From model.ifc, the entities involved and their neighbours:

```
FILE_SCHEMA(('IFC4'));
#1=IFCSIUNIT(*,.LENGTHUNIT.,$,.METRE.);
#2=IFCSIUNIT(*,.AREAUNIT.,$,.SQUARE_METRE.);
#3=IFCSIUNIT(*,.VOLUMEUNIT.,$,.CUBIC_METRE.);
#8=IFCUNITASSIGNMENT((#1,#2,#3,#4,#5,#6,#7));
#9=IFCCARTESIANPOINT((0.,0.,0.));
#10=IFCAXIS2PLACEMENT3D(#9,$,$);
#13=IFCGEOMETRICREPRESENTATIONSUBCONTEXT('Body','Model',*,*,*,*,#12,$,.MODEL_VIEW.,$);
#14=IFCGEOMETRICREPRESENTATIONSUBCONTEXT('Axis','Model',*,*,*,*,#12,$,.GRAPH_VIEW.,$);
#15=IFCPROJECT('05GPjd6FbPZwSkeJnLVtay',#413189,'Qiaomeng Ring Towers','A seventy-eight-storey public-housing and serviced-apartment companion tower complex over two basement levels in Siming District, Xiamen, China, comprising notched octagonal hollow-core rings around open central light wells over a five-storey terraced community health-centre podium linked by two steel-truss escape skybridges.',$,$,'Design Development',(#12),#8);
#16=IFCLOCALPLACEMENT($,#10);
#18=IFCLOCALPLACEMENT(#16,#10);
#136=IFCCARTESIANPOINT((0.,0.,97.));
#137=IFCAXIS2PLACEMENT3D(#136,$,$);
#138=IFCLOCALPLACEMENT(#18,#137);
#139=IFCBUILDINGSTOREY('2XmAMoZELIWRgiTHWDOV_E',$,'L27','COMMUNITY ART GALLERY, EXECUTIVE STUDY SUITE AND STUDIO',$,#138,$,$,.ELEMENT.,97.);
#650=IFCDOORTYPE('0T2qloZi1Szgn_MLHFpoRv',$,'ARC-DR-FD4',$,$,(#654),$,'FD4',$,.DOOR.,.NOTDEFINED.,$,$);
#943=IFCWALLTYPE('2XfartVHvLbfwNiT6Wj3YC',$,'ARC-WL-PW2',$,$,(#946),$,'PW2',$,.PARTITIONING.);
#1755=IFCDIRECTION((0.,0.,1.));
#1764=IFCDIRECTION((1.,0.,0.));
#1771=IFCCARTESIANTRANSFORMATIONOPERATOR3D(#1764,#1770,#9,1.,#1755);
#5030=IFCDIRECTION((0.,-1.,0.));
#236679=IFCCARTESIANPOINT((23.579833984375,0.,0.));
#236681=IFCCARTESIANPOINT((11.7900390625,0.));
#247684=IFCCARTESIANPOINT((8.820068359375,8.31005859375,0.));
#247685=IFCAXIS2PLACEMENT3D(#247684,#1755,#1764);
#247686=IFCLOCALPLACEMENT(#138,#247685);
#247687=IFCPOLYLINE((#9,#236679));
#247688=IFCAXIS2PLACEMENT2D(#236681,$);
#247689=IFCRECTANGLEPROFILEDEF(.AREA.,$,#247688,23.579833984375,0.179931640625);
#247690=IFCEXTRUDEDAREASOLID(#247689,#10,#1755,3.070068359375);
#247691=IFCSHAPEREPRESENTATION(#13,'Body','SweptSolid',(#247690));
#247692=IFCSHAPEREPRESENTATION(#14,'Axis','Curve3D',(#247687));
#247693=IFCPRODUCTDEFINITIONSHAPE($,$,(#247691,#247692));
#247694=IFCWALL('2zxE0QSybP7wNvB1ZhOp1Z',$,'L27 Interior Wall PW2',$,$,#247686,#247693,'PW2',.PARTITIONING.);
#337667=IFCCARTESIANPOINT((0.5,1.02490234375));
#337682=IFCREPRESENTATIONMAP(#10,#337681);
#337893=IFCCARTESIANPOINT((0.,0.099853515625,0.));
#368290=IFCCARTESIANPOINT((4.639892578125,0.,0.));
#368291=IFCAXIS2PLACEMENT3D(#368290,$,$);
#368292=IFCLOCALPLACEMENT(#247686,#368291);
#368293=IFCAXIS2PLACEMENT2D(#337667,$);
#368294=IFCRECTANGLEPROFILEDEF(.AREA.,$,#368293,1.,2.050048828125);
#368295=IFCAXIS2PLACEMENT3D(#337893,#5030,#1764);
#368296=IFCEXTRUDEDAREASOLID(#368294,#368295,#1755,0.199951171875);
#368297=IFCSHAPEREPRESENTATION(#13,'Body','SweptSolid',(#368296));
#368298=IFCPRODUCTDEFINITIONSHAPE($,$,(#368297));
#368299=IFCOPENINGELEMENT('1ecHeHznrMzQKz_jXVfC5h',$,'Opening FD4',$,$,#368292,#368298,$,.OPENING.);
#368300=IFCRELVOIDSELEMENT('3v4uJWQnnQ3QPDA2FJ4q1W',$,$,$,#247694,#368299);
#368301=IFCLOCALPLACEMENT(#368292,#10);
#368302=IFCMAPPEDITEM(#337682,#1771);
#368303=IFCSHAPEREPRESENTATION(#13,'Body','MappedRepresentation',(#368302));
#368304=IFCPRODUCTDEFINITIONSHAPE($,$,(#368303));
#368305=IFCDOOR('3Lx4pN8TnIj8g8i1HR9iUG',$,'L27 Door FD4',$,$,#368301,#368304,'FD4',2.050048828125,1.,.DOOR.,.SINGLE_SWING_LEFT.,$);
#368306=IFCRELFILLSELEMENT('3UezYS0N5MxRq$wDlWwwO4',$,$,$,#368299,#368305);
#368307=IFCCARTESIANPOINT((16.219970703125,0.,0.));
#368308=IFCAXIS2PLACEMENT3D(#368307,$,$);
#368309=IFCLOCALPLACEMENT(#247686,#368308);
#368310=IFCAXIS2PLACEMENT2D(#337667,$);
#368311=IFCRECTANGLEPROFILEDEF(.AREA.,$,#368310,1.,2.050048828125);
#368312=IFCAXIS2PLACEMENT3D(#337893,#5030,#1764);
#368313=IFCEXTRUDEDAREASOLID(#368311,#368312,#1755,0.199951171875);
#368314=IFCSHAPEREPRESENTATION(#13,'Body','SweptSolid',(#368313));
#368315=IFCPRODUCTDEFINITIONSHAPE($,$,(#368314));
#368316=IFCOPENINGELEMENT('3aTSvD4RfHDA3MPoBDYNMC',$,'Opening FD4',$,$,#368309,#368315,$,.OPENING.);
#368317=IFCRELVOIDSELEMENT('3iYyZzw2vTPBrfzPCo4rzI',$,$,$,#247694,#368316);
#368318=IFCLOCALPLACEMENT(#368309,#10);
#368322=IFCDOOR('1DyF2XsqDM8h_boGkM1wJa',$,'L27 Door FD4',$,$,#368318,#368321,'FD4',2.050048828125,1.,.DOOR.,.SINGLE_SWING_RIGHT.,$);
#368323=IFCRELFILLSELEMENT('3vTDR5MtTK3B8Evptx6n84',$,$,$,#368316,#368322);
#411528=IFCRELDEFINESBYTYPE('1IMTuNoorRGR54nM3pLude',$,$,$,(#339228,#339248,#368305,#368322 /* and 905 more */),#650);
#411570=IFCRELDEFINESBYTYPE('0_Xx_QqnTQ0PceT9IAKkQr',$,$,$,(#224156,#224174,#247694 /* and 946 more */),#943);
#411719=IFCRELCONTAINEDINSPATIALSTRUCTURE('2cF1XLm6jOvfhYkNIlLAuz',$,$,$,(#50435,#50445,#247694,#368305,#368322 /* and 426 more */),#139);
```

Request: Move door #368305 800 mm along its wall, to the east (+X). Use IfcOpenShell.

```python
import ifcopenshell
import ifcopenshell.api.geometry
import ifcopenshell.util.placement

model = ifcopenshell.open("model.ifc")

door = model.by_guid("3Lx4pN8TnIj8g8i1HR9iUG")
opening = door.FillsVoids[0].RelatingOpeningElement
wall = opening.VoidsElements[0].RelatingBuildingElement

wall_matrix = ifcopenshell.util.placement.get_local_placement(wall.ObjectPlacement)
shift = wall_matrix[:3, 0] * 0.8
before = ifcopenshell.util.placement.get_local_placement(door.ObjectPlacement)[:3, 3].copy()

# The door is placed relative to its opening, so it follows when the opening moves.
matrix = ifcopenshell.util.placement.get_local_placement(opening.ObjectPlacement)
matrix[:3, 3] += shift
ifcopenshell.api.geometry.edit_object_placement(
    model, product=opening, matrix=matrix, is_si=False, should_transform_children=True
)

after = ifcopenshell.util.placement.get_local_placement(door.ObjectPlacement)[:3, 3]
print("door moved by", (after - before).round(3) + 0.0)

model.write("model_v2.ifc")
```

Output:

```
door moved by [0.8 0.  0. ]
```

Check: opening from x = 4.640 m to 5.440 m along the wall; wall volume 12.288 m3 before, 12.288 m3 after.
